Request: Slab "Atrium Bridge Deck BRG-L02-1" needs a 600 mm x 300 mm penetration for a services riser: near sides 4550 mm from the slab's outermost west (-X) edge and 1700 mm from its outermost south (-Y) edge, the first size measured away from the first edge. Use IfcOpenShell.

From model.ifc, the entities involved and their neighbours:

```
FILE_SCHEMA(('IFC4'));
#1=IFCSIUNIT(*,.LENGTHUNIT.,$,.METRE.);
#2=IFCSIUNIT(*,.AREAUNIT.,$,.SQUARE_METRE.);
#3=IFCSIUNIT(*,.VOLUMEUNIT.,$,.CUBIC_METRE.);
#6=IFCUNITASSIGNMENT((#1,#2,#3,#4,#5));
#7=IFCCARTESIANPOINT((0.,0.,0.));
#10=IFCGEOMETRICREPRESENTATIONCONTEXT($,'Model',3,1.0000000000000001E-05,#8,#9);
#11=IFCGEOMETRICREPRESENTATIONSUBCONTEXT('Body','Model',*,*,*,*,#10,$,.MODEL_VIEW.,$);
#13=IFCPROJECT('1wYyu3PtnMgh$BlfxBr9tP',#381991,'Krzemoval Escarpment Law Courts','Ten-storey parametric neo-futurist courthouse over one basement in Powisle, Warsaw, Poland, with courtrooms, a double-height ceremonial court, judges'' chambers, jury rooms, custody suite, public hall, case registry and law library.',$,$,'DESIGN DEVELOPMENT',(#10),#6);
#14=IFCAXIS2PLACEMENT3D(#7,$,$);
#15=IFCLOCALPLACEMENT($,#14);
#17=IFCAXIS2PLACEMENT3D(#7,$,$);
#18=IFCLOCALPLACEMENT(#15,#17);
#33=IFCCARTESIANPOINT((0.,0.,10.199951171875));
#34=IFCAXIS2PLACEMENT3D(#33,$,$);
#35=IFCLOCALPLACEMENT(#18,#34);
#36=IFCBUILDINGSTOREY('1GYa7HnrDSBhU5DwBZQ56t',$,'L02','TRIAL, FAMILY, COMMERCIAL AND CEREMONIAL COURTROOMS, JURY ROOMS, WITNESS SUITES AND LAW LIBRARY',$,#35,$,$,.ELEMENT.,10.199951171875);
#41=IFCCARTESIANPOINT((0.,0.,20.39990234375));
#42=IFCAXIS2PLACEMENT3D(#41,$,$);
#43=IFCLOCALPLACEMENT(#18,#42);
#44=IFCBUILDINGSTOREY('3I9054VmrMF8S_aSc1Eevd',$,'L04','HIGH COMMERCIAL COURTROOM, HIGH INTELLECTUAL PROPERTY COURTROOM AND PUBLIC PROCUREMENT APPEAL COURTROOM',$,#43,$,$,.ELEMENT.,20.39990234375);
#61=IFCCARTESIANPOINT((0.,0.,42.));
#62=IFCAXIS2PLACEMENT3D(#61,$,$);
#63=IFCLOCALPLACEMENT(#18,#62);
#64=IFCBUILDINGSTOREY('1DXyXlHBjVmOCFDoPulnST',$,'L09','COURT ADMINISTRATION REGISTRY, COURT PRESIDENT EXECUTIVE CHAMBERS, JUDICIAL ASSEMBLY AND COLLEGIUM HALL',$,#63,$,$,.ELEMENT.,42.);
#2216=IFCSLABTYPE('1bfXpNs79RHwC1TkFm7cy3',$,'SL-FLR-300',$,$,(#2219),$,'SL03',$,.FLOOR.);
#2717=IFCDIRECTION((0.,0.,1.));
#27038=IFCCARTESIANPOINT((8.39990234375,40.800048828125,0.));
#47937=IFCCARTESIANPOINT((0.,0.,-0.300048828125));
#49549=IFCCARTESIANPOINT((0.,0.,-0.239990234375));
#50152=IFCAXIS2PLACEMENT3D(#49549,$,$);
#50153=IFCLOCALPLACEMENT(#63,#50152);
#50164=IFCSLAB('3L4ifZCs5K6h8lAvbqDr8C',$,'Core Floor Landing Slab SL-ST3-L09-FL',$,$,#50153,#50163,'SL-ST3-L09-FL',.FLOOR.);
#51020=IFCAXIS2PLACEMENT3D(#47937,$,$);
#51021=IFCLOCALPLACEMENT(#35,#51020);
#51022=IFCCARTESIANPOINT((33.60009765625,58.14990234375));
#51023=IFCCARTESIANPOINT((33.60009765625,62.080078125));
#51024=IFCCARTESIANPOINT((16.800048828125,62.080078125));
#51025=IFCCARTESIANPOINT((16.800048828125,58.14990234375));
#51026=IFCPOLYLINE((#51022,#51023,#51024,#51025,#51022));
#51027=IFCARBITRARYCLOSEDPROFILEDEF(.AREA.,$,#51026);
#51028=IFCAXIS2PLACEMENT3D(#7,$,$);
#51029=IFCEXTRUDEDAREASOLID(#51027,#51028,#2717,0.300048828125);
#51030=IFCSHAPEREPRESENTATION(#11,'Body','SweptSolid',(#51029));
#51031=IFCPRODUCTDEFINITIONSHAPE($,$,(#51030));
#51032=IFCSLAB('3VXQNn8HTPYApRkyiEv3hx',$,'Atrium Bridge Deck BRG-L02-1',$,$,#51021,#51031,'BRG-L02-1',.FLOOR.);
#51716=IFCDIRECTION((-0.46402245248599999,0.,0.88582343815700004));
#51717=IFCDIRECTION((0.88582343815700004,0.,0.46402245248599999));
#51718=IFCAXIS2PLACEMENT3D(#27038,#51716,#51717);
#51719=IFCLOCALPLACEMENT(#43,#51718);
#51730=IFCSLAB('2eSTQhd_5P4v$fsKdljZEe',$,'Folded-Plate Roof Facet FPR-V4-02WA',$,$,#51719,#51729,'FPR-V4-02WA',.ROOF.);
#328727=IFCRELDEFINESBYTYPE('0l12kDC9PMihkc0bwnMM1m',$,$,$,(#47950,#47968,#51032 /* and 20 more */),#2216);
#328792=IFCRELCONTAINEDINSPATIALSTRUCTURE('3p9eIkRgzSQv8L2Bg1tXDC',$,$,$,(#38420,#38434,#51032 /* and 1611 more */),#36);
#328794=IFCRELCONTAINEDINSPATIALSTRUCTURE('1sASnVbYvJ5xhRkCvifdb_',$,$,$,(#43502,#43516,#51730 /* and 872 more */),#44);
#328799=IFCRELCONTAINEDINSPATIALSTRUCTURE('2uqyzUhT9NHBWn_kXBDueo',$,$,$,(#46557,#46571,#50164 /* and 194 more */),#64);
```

```python
import numpy as np
import ifcopenshell
import ifcopenshell.api.feature
import ifcopenshell.api.geometry
import ifcopenshell.api.root
import ifcopenshell.geom
import ifcopenshell.util.placement
import ifcopenshell.util.representation
import ifcopenshell.util.shape
import ifcopenshell.util.unit

model = ifcopenshell.open("model.ifc")
unit_scale = ifcopenshell.util.unit.calculate_unit_scale(model)
settings = ifcopenshell.geom.settings()


def volume(element):
    """Net volume in cubic metres, openings subtracted."""
    shape = ifcopenshell.geom.create_shape(settings, element)
    return ifcopenshell.util.shape.get_volume(shape.geometry)


slab = model.by_guid("3VXQNn8HTPYApRkyiEv3hx")
before = volume(slab)

# Extent in the slab's own axes, in metres. The edges named are its -X and -Y sides.
slab_shape = ifcopenshell.geom.create_shape(settings, slab)
vertices = ifcopenshell.util.shape.get_vertices(slab_shape.geometry)
x_min, y_min, bottom = vertices.min(axis=0)
top = vertices[:, 2].max()

opening = ifcopenshell.api.root.create_entity(model, ifc_class="IfcOpeningElement", name="Services riser opening", predefined_type="OPENING")
context = ifcopenshell.util.representation.get_context(model, "Model", "Body", "MODEL_VIEW")
width, depth = 0.6, 0.3
outline = [(0.0, 0.0), (width, 0.0), (width, depth), (0.0, depth), (0.0, 0.0)]
# Overshoot both faces by 50 mm so the cut is clean.
shape = ifcopenshell.api.geometry.add_slab_representation(
    model, context=context, depth=top - bottom + 0.1, polyline=outline
)
ifcopenshell.api.geometry.assign_representation(model, product=opening, representation=shape)

matrix = ifcopenshell.util.placement.get_local_placement(slab.ObjectPlacement)
matrix[:, 3] = matrix @ np.append(np.array([x_min + 4.55, y_min + 1.7, bottom - 0.05]) / unit_scale, 1.0)
ifcopenshell.api.geometry.edit_object_placement(model, product=opening, matrix=matrix, is_si=False)
ifcopenshell.api.feature.add_feature(model, feature=opening, element=slab)

after = volume(slab)

print(f"slab volume {before:.3f} -> {after:.3f} m3")

model.write("model_edited.ifc")
```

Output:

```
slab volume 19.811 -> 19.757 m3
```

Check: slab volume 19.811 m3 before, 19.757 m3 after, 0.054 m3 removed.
